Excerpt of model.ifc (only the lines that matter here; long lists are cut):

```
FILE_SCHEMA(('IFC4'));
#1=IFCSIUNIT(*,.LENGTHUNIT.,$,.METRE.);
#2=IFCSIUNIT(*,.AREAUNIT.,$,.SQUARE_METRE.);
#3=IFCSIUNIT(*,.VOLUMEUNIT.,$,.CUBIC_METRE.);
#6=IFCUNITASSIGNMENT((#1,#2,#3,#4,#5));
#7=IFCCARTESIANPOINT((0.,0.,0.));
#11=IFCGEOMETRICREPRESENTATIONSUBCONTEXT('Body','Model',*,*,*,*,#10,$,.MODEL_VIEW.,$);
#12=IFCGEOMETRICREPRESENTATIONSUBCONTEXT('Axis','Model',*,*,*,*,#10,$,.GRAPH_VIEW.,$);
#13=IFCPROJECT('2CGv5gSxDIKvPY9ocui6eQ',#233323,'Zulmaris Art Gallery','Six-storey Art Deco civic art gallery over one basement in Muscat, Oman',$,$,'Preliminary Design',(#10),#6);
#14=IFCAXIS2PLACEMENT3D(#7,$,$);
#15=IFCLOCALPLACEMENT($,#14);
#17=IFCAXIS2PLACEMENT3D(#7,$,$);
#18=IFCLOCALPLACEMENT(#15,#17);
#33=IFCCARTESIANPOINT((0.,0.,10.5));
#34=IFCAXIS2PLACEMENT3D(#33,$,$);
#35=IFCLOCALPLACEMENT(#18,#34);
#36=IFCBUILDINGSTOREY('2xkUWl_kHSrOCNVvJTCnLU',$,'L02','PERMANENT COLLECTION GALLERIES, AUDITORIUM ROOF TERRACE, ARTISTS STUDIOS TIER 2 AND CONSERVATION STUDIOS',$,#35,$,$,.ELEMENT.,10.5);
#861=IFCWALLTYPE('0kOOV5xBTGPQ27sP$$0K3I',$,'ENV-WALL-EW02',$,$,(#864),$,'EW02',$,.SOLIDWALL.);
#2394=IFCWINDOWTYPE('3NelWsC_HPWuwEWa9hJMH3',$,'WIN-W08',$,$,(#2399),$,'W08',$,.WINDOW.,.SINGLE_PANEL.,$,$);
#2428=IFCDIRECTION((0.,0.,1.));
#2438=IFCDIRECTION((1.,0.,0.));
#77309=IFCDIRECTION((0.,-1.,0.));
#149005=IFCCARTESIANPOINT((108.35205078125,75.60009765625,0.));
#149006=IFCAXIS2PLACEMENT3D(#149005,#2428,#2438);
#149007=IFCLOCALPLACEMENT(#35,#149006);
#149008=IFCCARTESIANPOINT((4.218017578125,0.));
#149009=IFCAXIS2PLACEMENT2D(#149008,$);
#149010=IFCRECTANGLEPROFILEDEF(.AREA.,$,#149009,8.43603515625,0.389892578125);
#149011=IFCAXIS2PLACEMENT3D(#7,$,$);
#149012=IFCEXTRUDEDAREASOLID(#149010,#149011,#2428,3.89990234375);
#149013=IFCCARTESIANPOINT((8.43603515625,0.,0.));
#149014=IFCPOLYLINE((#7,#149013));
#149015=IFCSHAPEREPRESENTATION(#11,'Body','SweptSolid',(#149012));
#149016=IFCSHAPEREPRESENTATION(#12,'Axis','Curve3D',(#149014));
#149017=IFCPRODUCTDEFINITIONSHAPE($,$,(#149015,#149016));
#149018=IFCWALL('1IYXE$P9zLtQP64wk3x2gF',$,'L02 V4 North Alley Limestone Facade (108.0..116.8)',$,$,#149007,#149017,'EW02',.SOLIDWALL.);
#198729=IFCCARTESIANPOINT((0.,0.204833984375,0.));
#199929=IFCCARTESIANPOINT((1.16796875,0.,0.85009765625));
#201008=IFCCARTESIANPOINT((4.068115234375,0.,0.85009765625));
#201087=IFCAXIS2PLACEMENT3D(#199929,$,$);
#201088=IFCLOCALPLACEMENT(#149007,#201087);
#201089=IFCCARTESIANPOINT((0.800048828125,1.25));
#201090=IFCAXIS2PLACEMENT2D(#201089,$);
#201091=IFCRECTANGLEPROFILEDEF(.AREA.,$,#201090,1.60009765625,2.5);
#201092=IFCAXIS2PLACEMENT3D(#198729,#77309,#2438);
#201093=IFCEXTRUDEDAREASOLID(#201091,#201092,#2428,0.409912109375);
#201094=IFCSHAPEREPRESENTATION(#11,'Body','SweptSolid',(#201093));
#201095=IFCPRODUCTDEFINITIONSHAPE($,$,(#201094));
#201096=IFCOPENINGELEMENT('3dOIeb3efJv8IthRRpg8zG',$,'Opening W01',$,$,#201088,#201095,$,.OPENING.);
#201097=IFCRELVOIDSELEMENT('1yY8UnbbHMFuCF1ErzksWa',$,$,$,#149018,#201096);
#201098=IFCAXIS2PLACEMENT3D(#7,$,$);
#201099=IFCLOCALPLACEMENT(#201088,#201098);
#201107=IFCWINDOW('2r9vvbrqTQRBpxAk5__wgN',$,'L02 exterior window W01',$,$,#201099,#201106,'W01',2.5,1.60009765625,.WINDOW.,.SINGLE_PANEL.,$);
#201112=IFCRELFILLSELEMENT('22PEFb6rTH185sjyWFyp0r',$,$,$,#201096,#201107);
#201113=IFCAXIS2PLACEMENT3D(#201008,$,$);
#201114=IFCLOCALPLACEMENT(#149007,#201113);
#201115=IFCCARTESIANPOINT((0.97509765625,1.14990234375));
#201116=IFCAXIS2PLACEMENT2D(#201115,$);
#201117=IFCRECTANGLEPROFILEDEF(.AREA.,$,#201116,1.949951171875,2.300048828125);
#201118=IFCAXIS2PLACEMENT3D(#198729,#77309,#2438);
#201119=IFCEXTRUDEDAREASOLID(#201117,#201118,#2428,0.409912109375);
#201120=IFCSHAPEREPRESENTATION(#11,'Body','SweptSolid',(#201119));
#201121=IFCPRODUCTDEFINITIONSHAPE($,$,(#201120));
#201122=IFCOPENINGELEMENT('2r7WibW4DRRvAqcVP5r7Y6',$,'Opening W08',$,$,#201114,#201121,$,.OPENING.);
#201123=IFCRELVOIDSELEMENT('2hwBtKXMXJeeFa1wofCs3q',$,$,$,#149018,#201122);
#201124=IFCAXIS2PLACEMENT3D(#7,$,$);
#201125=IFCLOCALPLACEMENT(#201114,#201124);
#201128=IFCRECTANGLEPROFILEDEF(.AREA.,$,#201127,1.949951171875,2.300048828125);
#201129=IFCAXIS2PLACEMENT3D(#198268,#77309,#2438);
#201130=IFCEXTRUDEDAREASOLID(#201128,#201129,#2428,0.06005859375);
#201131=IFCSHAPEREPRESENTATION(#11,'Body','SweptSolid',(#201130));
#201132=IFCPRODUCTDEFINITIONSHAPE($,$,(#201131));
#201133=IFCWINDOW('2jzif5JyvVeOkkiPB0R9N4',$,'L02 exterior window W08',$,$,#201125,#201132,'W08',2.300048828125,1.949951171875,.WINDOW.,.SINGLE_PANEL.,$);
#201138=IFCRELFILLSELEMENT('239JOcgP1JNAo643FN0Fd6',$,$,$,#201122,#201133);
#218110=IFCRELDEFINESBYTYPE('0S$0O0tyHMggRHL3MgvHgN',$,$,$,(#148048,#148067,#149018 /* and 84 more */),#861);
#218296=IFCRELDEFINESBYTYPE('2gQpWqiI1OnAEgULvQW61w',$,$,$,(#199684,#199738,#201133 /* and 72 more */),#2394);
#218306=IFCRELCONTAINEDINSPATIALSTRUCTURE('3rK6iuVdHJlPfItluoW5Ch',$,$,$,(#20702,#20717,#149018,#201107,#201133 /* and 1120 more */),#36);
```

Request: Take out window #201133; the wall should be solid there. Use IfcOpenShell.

```python
import ifcopenshell
import ifcopenshell.api.feature
import ifcopenshell.api.root
import ifcopenshell.geom
import ifcopenshell.util.shape

model = ifcopenshell.open("model.ifc")
settings = ifcopenshell.geom.settings()


def volume(element):
    """Net volume in cubic metres, openings subtracted."""
    shape = ifcopenshell.geom.create_shape(settings, element)
    return ifcopenshell.util.shape.get_volume(shape.geometry)


window = model.by_guid("2jzif5JyvVeOkkiPB0R9N4")
opening = window.FillsVoids[0].RelatingOpeningElement
wall = opening.VoidsElements[0].RelatingBuildingElement
before = volume(wall)

ifcopenshell.api.root.remove_product(model, product=window)
ifcopenshell.api.feature.remove_feature(model, feature=opening)

after = volume(wall)

print(f"wall volume {before:.3f} -> {after:.3f} m3")

model.write("model_updated.ifc")
```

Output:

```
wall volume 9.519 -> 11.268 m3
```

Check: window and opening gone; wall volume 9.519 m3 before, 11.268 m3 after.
